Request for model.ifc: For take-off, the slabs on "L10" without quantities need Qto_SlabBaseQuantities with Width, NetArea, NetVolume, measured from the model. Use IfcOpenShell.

First a look at what the model holds.

```python
import ifcopenshell
import ifcopenshell.util.element
import ifcopenshell.util.unit

model = ifcopenshell.open("model.ifc")
print(model.schema)
for unit_type in ("LENGTHUNIT", "AREAUNIT", "VOLUMEUNIT"):
    print(unit_type, ifcopenshell.util.unit.calculate_unit_scale(model, unit_type))
storey = next(s for s in model.by_type("IfcBuildingStorey") if s.Name == "L10")
slabs = [e for e in ifcopenshell.util.element.get_decomposition(storey) if e.is_a("IfcSlab")]
for e in sorted(slabs, key=lambda e: e.id()):
    print(e.id(), e.is_a(), e.Name, list(ifcopenshell.util.element.get_psets(e, qtos_only=True)), sep=" | ")
```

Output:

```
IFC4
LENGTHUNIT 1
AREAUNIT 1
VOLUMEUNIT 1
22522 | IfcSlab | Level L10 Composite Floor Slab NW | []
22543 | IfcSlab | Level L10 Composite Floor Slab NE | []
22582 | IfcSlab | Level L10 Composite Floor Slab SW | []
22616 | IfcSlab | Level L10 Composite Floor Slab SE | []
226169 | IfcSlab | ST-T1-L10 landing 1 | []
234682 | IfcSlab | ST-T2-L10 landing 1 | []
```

```python
import ifcopenshell
import ifcopenshell.api.pset
import ifcopenshell.geom
import ifcopenshell.util.element
import ifcopenshell.util.shape
import ifcopenshell.util.unit

model = ifcopenshell.open("model.ifc")
unit_scale = ifcopenshell.util.unit.calculate_unit_scale(model)
area_scale = ifcopenshell.util.unit.calculate_unit_scale(model, "AREAUNIT")
volume_scale = ifcopenshell.util.unit.calculate_unit_scale(model, "VOLUMEUNIT")
settings = ifcopenshell.geom.settings()

storey = next(s for s in model.by_type("IfcBuildingStorey") if s.Name == "L10")
slabs = [e for e in ifcopenshell.util.element.get_decomposition(storey) if e.is_a("IfcSlab")]

for e in sorted(slabs, key=lambda e: e.id()):
    if ifcopenshell.util.element.get_psets(e, qtos_only=True, should_inherit=False):
        continue
    # Geometry comes back in metres, in the element's own axes.
    shape = ifcopenshell.geom.create_shape(settings, e)
    values = {
        "Width": ifcopenshell.util.shape.get_z(shape.geometry) / unit_scale,
        "NetArea": ifcopenshell.util.shape.get_footprint_area(shape.geometry) / area_scale,
        "NetVolume": ifcopenshell.util.shape.get_volume(shape.geometry) / volume_scale,
    }
    qto = ifcopenshell.api.pset.add_qto(model, product=e, name="Qto_SlabBaseQuantities")
    ifcopenshell.api.pset.edit_qto(model, qto=qto, properties=values)
    print(e.id(), {k: round(v, 3) for k, v in values.items()})

model.write("model_v2.ifc")
```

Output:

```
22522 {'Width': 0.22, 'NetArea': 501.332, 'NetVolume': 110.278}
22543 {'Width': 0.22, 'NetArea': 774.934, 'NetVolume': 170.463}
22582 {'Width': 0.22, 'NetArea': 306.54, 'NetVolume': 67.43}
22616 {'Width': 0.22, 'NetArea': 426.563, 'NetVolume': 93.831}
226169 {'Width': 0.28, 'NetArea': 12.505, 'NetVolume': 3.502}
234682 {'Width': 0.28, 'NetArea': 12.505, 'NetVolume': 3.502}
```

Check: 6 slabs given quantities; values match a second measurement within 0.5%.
